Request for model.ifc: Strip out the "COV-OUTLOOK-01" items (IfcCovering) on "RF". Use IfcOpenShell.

First a look at what the model holds.

```python
import ifcopenshell
import ifcopenshell.util.element

model = ifcopenshell.open("model.ifc")
print(model.schema)
storey = next(s for s in model.by_type("IfcBuildingStorey") if s.Name == "RF")
coverings = [e for e in ifcopenshell.util.element.get_decomposition(storey) if e.is_a("IfcCovering")]
seen = {}
for e in coverings:
    element_type = ifcopenshell.util.element.get_type(e)
    name = element_type.Name if element_type not in (None, e) else None
    seen[name] = seen.get(name, 0) + 1
for name, count in sorted(seen.items(), key=str):
    print(count, "x", name)
```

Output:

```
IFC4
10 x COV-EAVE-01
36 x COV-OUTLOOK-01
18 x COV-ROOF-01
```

```python
import ifcopenshell
import ifcopenshell.api.root
import ifcopenshell.util.element

model = ifcopenshell.open("model.ifc")

storey = next(s for s in model.by_type("IfcBuildingStorey") if s.Name == "RF")
coverings = [e for e in ifcopenshell.util.element.get_decomposition(storey) if e.is_a("IfcCovering")]
targets = [e for e in coverings if (t := ifcopenshell.util.element.get_type(e)) not in (None, e) and t.Name == "COV-OUTLOOK-01"]

for e in targets:
    ifcopenshell.api.root.remove_product(model, product=e)
print(len(targets), "removed")

model.write("model-out.ifc")
```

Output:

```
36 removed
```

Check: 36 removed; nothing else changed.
